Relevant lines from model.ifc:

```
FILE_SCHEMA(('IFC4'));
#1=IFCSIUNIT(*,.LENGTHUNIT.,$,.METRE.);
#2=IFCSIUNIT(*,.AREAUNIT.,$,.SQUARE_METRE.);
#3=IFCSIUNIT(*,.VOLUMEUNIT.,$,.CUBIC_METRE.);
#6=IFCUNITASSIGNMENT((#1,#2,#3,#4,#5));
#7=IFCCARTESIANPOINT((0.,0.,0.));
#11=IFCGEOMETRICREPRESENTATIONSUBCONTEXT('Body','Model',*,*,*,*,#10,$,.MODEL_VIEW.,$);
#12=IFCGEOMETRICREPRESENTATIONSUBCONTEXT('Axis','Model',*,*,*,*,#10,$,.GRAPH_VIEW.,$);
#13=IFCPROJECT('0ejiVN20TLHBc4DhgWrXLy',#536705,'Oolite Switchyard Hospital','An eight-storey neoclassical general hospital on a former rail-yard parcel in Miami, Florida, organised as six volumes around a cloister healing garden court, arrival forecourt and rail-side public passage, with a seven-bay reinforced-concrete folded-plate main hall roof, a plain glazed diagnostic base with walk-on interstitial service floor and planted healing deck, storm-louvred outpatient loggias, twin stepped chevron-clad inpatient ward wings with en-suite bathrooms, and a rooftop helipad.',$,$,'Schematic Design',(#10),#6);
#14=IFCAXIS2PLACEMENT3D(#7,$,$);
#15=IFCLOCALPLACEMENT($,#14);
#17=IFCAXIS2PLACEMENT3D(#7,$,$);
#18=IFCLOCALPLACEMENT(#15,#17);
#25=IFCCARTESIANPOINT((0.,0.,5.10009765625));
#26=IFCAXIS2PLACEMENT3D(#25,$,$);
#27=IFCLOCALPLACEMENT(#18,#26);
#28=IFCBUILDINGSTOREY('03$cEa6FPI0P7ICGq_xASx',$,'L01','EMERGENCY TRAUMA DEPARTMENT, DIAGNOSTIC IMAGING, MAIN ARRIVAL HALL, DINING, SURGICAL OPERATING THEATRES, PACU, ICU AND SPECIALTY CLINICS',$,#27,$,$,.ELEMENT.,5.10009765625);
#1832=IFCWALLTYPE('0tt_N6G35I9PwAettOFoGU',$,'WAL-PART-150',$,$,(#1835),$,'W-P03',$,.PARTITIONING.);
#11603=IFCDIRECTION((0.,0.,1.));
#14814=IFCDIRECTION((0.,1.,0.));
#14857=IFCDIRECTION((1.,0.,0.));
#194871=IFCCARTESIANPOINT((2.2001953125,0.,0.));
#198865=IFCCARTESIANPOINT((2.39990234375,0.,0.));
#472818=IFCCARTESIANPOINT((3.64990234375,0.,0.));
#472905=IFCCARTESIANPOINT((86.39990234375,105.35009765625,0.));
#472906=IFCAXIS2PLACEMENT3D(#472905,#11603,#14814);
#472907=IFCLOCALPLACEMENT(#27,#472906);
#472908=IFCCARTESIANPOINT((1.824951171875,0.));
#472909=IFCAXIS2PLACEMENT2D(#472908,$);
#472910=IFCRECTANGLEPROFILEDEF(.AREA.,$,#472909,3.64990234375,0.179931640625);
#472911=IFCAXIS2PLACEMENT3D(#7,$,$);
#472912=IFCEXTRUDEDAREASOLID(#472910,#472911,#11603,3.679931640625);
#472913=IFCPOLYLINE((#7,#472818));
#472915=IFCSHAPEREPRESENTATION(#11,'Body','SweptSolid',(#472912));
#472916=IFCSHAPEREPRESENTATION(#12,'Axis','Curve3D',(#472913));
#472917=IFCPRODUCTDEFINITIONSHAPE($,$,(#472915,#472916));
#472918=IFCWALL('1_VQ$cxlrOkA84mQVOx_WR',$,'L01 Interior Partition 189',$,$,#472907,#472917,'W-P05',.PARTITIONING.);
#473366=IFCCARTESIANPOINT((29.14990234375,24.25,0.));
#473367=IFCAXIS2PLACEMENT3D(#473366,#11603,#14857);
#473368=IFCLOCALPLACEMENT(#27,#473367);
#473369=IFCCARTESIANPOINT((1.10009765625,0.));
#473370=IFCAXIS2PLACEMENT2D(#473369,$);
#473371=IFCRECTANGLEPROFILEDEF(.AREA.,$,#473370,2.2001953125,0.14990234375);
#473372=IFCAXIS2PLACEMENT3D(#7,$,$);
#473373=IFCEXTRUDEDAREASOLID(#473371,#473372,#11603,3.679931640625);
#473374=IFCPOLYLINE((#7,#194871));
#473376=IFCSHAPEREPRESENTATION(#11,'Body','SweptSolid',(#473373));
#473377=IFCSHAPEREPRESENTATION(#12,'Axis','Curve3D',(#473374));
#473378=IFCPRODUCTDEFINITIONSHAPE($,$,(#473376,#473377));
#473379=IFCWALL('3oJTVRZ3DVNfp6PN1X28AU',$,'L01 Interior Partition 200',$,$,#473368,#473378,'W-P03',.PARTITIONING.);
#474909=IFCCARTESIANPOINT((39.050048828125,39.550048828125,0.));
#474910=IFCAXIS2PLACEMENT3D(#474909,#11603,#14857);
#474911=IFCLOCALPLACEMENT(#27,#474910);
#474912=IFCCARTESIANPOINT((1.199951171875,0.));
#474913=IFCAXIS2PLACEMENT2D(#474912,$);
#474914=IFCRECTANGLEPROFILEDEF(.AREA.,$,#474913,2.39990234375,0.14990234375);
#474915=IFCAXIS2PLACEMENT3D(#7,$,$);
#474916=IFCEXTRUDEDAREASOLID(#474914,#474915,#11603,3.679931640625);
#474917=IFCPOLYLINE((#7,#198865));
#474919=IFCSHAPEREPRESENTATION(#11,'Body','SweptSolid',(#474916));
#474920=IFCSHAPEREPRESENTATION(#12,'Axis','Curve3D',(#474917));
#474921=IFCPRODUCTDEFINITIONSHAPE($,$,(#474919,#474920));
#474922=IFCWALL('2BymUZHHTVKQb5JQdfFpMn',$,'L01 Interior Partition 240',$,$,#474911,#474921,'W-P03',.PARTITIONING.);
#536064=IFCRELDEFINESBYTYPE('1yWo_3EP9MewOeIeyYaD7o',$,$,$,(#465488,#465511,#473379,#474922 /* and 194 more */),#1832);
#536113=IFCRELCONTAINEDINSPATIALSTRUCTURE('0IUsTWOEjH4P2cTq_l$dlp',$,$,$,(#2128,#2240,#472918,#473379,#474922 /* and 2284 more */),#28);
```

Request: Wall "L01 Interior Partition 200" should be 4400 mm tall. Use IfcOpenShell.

```python
import ifcopenshell
import ifcopenshell.geom
import ifcopenshell.util.representation
import ifcopenshell.util.shape
import ifcopenshell.util.unit

model = ifcopenshell.open("model.ifc")
unit_scale = ifcopenshell.util.unit.calculate_unit_scale(model)
settings = ifcopenshell.geom.settings()


def volume(element):
    """Net volume in cubic metres, openings subtracted."""
    shape = ifcopenshell.geom.create_shape(settings, element)
    return ifcopenshell.util.shape.get_volume(shape.geometry)


wall = model.by_guid("3oJTVRZ3DVNfp6PN1X28AU")
before = volume(wall)

body = ifcopenshell.util.representation.get_representation(wall, "Model", "Body")
solid = body.Items[0]
old_height = solid.Depth
solid.Depth = 4.4 / unit_scale
after = volume(wall)

print(f"height {old_height:g} -> {solid.Depth:g}, volume {before:.3f} -> {after:.3f} m3")

model.write("model_updated.ifc")
```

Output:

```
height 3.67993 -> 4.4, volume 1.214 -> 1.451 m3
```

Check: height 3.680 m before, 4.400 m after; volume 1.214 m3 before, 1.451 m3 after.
